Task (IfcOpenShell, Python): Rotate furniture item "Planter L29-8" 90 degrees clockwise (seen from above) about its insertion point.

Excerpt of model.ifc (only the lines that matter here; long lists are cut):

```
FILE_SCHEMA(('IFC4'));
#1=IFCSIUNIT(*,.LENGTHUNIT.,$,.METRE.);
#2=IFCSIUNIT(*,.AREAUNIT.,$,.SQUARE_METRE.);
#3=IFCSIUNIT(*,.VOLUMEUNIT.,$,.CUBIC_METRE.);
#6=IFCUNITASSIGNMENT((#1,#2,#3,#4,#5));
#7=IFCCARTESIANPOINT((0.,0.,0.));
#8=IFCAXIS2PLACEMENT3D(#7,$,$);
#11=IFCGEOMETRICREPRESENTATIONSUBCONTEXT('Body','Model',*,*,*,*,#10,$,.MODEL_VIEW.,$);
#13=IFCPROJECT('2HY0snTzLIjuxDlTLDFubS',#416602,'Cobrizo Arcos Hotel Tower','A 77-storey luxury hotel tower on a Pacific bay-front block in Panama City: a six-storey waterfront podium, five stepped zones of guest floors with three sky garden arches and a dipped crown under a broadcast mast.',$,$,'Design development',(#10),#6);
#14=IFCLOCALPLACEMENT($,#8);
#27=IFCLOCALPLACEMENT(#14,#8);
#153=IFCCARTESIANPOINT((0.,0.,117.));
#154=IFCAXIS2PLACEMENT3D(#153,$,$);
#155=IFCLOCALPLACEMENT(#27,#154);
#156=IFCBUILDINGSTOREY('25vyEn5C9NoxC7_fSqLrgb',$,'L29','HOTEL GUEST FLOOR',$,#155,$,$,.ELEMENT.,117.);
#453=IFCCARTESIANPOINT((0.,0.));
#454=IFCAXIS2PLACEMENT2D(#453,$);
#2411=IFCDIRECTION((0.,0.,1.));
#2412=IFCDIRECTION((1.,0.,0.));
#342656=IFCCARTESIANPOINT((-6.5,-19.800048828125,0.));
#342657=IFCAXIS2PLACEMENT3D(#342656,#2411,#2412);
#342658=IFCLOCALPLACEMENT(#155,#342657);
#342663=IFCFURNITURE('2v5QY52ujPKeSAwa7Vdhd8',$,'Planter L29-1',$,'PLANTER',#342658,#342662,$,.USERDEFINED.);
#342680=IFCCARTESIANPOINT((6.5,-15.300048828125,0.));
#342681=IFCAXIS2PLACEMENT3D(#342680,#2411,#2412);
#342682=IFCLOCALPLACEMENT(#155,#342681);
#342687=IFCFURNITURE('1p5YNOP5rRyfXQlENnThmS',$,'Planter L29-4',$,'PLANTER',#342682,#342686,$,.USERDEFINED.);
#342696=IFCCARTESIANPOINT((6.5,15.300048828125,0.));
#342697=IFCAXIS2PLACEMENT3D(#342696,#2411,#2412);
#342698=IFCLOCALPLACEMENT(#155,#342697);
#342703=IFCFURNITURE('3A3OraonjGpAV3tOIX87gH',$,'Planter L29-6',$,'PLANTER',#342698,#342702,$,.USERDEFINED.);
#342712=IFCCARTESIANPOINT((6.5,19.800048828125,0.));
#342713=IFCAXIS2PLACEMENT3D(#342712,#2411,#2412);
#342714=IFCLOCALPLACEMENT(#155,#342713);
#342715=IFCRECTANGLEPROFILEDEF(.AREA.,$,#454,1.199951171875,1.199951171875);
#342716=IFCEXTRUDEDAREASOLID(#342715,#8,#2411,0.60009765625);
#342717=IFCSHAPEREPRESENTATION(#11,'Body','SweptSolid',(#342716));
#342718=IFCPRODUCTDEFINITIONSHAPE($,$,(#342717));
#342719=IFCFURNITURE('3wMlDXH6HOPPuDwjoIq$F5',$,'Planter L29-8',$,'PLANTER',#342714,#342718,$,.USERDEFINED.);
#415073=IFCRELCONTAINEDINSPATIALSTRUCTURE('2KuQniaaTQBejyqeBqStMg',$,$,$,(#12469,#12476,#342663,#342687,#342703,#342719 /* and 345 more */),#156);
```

```python
import ifcopenshell
import ifcopenshell.api.geometry
import ifcopenshell.util.placement

model = ifcopenshell.open("model.ifc")

item = model.by_guid("3wMlDXH6HOPPuDwjoIq$F5")
matrix = ifcopenshell.util.placement.get_local_placement(item.ObjectPlacement)
matrix = matrix @ ifcopenshell.util.placement.rotation(-90, "Z")
ifcopenshell.api.geometry.edit_object_placement(model, product=item, matrix=matrix, is_si=False)

print(ifcopenshell.util.placement.get_local_placement(item.ObjectPlacement).round(3) + 0.0)

model.write("model_rev.ifc")
```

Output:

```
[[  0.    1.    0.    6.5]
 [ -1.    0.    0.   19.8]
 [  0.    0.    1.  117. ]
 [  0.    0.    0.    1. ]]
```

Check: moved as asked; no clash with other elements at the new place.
